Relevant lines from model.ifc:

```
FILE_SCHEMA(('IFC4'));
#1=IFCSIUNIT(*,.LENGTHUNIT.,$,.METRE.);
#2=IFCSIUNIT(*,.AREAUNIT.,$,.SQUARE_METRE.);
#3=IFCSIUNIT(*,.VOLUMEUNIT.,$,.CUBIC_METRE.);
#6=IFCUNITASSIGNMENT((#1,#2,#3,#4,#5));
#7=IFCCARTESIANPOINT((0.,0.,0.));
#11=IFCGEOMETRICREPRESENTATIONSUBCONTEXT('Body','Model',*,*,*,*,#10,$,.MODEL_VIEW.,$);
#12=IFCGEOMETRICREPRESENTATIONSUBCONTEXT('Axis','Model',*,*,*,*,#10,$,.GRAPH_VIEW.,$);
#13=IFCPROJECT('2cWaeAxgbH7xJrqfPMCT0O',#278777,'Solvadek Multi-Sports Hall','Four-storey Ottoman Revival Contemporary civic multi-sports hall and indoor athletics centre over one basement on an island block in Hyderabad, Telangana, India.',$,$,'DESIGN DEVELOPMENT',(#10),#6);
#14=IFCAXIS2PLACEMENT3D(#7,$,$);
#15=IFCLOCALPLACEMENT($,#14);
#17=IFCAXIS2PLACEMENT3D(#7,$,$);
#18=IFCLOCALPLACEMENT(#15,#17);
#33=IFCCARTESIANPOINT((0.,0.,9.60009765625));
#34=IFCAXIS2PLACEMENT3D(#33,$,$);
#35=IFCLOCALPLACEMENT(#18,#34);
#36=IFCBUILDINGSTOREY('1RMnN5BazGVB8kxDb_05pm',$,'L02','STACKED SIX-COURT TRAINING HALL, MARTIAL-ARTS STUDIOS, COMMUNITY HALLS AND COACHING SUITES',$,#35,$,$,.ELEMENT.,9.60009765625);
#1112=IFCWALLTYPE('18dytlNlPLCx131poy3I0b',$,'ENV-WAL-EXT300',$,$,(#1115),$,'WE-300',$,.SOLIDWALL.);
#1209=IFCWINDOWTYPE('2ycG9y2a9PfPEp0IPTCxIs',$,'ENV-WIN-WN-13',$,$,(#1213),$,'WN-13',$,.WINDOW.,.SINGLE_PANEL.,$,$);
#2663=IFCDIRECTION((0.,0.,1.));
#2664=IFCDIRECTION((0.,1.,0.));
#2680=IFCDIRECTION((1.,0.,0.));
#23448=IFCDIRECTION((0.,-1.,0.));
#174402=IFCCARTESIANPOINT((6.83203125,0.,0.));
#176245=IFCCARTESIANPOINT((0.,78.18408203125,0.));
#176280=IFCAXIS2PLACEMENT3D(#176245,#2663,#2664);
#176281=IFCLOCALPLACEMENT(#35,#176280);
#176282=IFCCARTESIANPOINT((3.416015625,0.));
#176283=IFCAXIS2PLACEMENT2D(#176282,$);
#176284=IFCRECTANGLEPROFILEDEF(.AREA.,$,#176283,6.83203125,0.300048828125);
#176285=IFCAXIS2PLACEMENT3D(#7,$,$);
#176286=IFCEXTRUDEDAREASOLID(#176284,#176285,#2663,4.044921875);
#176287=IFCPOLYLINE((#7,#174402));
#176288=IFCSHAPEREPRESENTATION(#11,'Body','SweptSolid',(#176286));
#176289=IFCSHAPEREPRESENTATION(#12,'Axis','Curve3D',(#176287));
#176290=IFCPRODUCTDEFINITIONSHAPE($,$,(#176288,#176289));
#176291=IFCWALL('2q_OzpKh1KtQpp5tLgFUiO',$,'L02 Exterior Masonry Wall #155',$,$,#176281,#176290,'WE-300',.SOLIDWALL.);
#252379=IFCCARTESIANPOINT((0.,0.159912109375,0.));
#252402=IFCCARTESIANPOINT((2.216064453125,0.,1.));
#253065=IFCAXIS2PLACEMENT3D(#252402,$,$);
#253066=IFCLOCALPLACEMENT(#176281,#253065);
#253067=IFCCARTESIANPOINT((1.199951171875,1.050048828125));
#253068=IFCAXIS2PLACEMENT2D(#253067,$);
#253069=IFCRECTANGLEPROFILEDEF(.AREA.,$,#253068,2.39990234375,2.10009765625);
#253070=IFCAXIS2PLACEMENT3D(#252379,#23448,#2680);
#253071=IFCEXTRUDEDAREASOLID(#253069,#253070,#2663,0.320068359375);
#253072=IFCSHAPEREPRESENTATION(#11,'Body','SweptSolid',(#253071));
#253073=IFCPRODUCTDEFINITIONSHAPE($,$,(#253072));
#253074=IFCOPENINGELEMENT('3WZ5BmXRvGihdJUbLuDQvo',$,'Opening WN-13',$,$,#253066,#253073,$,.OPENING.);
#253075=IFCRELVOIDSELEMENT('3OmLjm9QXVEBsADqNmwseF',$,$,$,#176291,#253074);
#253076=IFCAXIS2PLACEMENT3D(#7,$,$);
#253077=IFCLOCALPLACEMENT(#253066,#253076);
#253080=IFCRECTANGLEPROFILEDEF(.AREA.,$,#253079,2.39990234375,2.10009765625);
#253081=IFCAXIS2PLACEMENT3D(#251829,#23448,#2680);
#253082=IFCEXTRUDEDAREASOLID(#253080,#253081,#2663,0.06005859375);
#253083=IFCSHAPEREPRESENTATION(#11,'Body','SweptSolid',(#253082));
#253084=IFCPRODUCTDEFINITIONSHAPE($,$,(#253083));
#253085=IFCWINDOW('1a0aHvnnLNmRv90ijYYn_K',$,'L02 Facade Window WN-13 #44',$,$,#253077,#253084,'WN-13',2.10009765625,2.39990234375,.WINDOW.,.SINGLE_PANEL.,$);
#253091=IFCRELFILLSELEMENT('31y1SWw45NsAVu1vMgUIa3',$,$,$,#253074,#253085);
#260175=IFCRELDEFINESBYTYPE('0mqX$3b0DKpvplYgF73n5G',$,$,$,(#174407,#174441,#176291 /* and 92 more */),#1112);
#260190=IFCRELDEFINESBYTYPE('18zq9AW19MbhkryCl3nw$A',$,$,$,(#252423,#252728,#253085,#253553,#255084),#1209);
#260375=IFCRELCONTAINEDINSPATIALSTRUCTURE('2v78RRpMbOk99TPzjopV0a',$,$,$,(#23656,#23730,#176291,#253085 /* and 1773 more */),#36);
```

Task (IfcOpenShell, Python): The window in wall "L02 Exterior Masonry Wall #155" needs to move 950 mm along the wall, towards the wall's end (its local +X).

```python
import ifcopenshell
import ifcopenshell.api.geometry
import ifcopenshell.util.placement
import ifcopenshell.util.unit

model = ifcopenshell.open("model.ifc")
unit_scale = ifcopenshell.util.unit.calculate_unit_scale(model)

window = model.by_id(253085)
opening = window.FillsVoids[0].RelatingOpeningElement
wall = opening.VoidsElements[0].RelatingBuildingElement

wall_matrix = ifcopenshell.util.placement.get_local_placement(wall.ObjectPlacement)
shift = wall_matrix[:3, 0] * 0.95 / unit_scale
before = ifcopenshell.util.placement.get_local_placement(window.ObjectPlacement)[:3, 3].copy()

# The window is placed relative to its opening, so it follows when the opening moves.
matrix = ifcopenshell.util.placement.get_local_placement(opening.ObjectPlacement)
matrix[:3, 3] += shift
ifcopenshell.api.geometry.edit_object_placement(
    model, product=opening, matrix=matrix, is_si=False, should_transform_children=True
)

after = ifcopenshell.util.placement.get_local_placement(window.ObjectPlacement)[:3, 3]
print("window moved by", (after - before).round(3) + 0.0)

model.write("model-out.ifc")
```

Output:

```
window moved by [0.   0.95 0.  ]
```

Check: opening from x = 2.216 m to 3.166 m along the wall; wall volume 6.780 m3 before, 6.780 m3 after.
